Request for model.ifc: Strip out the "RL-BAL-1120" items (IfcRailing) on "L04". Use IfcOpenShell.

First a look at what the model holds.

```python
import ifcopenshell
import ifcopenshell.util.element

model = ifcopenshell.open("model.ifc")
print(model.schema)
storey = next(s for s in model.by_type("IfcBuildingStorey") if s.Name == "L04")
railings = [e for e in ifcopenshell.util.element.get_decomposition(storey) if e.is_a("IfcRailing")]
seen = {}
for e in railings:
    element_type = ifcopenshell.util.element.get_type(e)
    name = element_type.Name if element_type not in (None, e) else None
    seen[name] = seen.get(name, 0) + 1
for name, count in sorted(seen.items(), key=str):
    print(count, "x", name)
```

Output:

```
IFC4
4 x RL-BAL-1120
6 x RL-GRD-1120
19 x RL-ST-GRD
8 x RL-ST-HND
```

```python
import ifcopenshell
import ifcopenshell.api.root
import ifcopenshell.util.element

model = ifcopenshell.open("model.ifc")

storey = next(s for s in model.by_type("IfcBuildingStorey") if s.Name == "L04")
railings = [e for e in ifcopenshell.util.element.get_decomposition(storey) if e.is_a("IfcRailing")]
targets = [e for e in railings if (t := ifcopenshell.util.element.get_type(e)) not in (None, e) and t.Name == "RL-BAL-1120"]

for e in targets:
    ifcopenshell.api.root.remove_product(model, product=e)
print(len(targets), "removed")

model.write("model-out.ifc")
```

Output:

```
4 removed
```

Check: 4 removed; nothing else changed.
